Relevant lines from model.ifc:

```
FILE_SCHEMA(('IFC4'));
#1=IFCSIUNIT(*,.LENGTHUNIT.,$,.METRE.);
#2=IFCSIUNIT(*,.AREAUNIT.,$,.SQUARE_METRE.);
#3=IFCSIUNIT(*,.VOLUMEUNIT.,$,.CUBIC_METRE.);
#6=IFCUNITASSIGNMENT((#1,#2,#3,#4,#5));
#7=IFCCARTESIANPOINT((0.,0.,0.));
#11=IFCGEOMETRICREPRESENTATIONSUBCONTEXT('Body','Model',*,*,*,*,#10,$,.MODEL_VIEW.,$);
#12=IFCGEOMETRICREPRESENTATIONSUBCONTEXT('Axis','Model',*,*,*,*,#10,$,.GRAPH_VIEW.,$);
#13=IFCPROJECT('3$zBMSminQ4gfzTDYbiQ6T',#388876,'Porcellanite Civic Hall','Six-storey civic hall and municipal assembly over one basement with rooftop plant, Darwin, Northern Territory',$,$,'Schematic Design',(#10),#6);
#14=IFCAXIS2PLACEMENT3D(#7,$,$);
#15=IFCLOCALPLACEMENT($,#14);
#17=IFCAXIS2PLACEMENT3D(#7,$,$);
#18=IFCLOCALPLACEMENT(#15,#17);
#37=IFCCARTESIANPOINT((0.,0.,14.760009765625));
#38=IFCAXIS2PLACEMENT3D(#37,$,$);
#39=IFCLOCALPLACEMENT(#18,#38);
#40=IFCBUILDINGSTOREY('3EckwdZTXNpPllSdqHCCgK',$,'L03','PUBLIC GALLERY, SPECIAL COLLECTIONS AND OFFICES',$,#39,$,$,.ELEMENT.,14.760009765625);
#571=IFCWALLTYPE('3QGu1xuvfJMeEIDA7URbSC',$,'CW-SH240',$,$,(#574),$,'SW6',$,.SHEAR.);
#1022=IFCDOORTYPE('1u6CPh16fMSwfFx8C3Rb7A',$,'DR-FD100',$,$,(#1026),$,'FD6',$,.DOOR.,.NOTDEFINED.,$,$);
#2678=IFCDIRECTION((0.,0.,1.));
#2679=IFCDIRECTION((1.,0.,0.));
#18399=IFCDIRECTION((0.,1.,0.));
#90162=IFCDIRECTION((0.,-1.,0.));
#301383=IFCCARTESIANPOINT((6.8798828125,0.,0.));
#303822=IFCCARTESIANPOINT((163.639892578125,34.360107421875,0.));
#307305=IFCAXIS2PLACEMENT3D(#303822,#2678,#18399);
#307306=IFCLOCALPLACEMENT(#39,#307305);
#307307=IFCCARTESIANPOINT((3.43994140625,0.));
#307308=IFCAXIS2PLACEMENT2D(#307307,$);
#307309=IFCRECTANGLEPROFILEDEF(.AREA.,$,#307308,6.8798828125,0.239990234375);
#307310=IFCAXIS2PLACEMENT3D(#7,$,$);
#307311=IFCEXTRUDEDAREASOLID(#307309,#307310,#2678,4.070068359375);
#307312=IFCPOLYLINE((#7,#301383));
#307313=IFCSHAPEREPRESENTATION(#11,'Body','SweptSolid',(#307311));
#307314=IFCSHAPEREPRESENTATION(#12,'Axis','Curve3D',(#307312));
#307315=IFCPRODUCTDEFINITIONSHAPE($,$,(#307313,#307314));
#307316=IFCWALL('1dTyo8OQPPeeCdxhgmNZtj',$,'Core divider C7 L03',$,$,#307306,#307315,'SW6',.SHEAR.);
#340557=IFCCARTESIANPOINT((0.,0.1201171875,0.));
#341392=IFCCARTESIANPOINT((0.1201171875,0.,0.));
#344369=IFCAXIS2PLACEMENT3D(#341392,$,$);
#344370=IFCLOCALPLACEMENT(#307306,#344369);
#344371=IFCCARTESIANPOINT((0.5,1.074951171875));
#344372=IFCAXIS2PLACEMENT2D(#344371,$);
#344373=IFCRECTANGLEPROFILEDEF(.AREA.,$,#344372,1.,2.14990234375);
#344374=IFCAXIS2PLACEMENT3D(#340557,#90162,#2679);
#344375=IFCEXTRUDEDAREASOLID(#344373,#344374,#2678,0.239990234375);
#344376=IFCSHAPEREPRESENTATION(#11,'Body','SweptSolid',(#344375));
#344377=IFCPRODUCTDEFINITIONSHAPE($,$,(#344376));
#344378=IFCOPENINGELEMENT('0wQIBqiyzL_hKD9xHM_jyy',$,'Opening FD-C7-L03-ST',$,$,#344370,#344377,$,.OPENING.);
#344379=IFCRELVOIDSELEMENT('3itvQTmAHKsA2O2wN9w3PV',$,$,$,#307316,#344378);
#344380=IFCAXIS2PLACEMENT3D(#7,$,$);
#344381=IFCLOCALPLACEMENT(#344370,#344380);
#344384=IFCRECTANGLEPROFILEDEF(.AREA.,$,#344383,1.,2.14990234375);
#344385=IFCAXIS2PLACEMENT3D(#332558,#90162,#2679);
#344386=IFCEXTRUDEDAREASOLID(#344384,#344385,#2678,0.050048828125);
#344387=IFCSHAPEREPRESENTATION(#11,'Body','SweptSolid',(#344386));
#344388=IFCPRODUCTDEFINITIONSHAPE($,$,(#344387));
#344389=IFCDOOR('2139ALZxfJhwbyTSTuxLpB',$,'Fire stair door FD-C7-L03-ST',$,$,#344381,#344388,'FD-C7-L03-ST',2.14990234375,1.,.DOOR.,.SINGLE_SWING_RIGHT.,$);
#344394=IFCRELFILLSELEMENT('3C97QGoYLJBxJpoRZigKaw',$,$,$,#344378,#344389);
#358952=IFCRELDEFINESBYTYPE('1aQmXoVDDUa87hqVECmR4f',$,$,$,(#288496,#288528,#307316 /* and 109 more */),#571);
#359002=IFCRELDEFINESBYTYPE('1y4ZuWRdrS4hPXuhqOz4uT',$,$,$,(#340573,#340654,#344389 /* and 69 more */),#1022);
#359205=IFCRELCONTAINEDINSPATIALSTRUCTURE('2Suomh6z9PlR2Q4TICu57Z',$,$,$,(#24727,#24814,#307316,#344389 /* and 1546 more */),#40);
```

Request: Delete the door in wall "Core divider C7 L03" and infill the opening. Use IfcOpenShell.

```python
import ifcopenshell
import ifcopenshell.api.feature
import ifcopenshell.api.root
import ifcopenshell.geom
import ifcopenshell.util.shape

model = ifcopenshell.open("model.ifc")
settings = ifcopenshell.geom.settings()


def volume(element):
    """Net volume in cubic metres, openings subtracted."""
    shape = ifcopenshell.geom.create_shape(settings, element)
    return ifcopenshell.util.shape.get_volume(shape.geometry)


door = model.by_id(344389)
opening = door.FillsVoids[0].RelatingOpeningElement
wall = opening.VoidsElements[0].RelatingBuildingElement
before = volume(wall)

ifcopenshell.api.root.remove_product(model, product=door)
ifcopenshell.api.feature.remove_feature(model, feature=opening)

after = volume(wall)

print(f"wall volume {before:.3f} -> {after:.3f} m3")

model.write("model_updated.ifc")
```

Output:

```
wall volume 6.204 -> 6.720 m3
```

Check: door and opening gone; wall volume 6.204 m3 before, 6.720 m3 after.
